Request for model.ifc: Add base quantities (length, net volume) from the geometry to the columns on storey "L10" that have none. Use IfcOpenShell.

First a look at what the model holds.

```python
import ifcopenshell
import ifcopenshell.util.element
import ifcopenshell.util.unit

model = ifcopenshell.open("model.ifc")
print(model.schema)
for unit_type in ("LENGTHUNIT", "AREAUNIT", "VOLUMEUNIT"):
    print(unit_type, ifcopenshell.util.unit.calculate_unit_scale(model, unit_type))
storey = next(s for s in model.by_type("IfcBuildingStorey") if s.Name == "L10")
columns = [e for e in ifcopenshell.util.element.get_decomposition(storey) if e.is_a("IfcColumn")]
for e in sorted(columns, key=lambda e: e.id()):
    print(e.id(), e.is_a(), e.Name, list(ifcopenshell.util.element.get_psets(e, qtos_only=True)), sep=" | ")
```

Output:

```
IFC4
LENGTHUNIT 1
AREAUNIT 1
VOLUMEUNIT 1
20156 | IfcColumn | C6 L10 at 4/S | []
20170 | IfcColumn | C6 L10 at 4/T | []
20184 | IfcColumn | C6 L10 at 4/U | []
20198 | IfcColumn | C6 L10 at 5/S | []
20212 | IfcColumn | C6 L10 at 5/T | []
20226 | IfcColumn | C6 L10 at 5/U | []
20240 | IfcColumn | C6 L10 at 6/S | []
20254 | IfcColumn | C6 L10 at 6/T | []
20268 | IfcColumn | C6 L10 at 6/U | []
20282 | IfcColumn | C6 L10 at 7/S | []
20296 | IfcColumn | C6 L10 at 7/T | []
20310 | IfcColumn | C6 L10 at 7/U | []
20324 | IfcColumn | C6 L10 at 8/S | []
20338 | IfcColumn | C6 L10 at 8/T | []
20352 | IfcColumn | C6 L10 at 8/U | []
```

```python
import ifcopenshell
import ifcopenshell.api.pset
import ifcopenshell.geom
import ifcopenshell.util.element
import ifcopenshell.util.shape
import ifcopenshell.util.unit

model = ifcopenshell.open("model.ifc")
unit_scale = ifcopenshell.util.unit.calculate_unit_scale(model)
volume_scale = ifcopenshell.util.unit.calculate_unit_scale(model, "VOLUMEUNIT")
settings = ifcopenshell.geom.settings()

storey = next(s for s in model.by_type("IfcBuildingStorey") if s.Name == "L10")
columns = [e for e in ifcopenshell.util.element.get_decomposition(storey) if e.is_a("IfcColumn")]

for e in sorted(columns, key=lambda e: e.id()):
    if ifcopenshell.util.element.get_psets(e, qtos_only=True, should_inherit=False):
        continue
    # Geometry comes back in metres, in the element's own axes.
    shape = ifcopenshell.geom.create_shape(settings, e)
    values = {
        "Length": ifcopenshell.util.shape.get_z(shape.geometry) / unit_scale,
        "NetVolume": ifcopenshell.util.shape.get_volume(shape.geometry) / volume_scale,
    }
    qto = ifcopenshell.api.pset.add_qto(model, product=e, name="Qto_ColumnBaseQuantities")
    ifcopenshell.api.pset.edit_qto(model, qto=qto, properties=values)
    print(e.id(), {k: round(v, 3) for k, v in values.items()})

model.write("model-out.ifc")
```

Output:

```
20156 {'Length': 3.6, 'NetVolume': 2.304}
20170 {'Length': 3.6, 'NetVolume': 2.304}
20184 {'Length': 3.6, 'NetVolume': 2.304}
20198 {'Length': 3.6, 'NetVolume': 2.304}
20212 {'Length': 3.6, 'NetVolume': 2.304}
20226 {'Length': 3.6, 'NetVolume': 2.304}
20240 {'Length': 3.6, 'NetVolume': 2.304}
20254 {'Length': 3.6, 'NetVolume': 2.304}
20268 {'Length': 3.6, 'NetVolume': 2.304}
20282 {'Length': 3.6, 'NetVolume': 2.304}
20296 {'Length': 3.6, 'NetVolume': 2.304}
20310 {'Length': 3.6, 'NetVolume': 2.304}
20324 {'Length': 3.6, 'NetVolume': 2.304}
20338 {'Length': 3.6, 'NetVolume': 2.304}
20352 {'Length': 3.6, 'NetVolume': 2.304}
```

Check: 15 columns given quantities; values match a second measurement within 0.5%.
